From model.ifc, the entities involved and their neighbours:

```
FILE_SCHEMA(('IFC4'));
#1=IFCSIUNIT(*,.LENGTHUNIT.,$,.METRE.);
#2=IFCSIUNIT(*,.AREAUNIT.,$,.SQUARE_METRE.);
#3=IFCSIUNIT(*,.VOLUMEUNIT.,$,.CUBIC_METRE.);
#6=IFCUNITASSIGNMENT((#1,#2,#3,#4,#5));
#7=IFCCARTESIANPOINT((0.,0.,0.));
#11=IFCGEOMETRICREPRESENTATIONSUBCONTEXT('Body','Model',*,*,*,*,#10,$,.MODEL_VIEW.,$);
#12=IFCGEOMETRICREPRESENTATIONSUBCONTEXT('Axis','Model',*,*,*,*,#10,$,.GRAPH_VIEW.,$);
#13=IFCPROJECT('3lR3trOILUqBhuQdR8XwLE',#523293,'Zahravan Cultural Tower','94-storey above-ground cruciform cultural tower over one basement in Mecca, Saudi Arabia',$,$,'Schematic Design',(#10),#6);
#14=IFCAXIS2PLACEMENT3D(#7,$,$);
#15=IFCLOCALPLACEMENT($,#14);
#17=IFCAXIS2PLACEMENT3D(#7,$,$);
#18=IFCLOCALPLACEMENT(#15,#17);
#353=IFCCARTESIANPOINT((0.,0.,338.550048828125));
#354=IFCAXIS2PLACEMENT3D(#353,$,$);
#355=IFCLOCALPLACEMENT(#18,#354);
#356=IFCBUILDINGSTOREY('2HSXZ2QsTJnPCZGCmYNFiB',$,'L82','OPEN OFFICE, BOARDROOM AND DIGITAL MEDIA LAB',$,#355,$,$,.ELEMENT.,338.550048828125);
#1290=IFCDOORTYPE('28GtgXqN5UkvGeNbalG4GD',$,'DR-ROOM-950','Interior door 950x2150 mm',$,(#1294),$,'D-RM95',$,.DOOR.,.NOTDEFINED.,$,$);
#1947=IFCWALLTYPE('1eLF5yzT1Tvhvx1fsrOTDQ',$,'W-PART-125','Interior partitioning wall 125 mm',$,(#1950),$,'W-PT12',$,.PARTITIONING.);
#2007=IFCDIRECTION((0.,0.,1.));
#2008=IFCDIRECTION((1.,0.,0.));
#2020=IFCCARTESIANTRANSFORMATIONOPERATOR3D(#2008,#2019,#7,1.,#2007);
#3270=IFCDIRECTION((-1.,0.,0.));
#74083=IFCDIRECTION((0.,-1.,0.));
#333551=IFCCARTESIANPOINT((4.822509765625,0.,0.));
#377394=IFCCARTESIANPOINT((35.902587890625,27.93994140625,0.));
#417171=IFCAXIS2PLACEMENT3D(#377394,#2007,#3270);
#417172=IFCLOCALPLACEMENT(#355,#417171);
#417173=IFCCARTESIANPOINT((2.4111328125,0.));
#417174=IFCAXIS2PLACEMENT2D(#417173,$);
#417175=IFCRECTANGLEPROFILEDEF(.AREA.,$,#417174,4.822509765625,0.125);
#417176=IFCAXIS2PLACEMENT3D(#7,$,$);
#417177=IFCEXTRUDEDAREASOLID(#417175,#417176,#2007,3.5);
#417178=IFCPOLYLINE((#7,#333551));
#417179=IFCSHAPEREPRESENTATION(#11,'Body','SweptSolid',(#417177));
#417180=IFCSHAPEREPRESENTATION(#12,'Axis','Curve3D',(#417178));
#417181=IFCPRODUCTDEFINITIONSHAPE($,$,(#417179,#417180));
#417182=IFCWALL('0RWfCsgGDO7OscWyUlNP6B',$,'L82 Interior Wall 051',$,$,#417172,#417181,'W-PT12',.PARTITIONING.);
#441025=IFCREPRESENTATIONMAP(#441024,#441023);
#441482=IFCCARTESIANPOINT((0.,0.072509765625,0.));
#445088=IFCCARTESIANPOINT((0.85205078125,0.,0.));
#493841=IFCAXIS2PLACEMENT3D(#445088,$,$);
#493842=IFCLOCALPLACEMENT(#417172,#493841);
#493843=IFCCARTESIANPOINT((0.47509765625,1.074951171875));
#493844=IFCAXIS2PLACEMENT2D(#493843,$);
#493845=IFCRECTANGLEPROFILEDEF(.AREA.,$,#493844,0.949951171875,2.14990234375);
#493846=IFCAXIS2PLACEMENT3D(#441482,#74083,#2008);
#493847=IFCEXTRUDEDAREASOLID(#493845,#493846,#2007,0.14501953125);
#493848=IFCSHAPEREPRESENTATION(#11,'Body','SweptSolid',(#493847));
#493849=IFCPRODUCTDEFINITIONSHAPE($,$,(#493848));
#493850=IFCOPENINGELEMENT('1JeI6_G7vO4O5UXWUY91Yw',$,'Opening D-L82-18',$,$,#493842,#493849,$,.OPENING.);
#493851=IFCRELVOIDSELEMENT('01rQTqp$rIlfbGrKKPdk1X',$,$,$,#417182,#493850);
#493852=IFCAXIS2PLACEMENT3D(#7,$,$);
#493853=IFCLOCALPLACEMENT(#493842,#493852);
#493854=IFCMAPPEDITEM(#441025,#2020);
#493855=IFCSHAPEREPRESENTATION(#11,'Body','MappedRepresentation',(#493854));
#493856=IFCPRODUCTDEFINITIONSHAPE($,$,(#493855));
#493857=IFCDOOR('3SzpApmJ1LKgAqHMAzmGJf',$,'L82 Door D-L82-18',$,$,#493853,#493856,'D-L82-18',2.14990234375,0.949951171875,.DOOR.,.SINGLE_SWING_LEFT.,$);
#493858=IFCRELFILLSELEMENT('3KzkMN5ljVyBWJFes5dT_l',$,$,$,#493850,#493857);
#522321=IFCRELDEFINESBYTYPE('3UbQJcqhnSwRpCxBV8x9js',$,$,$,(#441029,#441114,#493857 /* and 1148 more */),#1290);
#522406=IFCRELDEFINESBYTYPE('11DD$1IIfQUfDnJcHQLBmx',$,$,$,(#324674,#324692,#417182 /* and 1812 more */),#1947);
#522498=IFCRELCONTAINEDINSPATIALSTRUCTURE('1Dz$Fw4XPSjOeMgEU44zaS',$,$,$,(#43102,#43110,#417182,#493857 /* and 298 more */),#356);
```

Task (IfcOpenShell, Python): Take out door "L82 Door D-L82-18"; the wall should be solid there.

```python
import ifcopenshell
import ifcopenshell.api.feature
import ifcopenshell.api.root
import ifcopenshell.geom
import ifcopenshell.util.shape

model = ifcopenshell.open("model.ifc")
settings = ifcopenshell.geom.settings()


def volume(element):
    """Net volume in cubic metres, openings subtracted."""
    shape = ifcopenshell.geom.create_shape(settings, element)
    return ifcopenshell.util.shape.get_volume(shape.geometry)


door = model.by_guid("3SzpApmJ1LKgAqHMAzmGJf")
opening = door.FillsVoids[0].RelatingOpeningElement
wall = opening.VoidsElements[0].RelatingBuildingElement
before = volume(wall)

ifcopenshell.api.root.remove_product(model, product=door)
ifcopenshell.api.feature.remove_feature(model, feature=opening)

after = volume(wall)

print(f"wall volume {before:.3f} -> {after:.3f} m3")

model.write("model_v2.ifc")
```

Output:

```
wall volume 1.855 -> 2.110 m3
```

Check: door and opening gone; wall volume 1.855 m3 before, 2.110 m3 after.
